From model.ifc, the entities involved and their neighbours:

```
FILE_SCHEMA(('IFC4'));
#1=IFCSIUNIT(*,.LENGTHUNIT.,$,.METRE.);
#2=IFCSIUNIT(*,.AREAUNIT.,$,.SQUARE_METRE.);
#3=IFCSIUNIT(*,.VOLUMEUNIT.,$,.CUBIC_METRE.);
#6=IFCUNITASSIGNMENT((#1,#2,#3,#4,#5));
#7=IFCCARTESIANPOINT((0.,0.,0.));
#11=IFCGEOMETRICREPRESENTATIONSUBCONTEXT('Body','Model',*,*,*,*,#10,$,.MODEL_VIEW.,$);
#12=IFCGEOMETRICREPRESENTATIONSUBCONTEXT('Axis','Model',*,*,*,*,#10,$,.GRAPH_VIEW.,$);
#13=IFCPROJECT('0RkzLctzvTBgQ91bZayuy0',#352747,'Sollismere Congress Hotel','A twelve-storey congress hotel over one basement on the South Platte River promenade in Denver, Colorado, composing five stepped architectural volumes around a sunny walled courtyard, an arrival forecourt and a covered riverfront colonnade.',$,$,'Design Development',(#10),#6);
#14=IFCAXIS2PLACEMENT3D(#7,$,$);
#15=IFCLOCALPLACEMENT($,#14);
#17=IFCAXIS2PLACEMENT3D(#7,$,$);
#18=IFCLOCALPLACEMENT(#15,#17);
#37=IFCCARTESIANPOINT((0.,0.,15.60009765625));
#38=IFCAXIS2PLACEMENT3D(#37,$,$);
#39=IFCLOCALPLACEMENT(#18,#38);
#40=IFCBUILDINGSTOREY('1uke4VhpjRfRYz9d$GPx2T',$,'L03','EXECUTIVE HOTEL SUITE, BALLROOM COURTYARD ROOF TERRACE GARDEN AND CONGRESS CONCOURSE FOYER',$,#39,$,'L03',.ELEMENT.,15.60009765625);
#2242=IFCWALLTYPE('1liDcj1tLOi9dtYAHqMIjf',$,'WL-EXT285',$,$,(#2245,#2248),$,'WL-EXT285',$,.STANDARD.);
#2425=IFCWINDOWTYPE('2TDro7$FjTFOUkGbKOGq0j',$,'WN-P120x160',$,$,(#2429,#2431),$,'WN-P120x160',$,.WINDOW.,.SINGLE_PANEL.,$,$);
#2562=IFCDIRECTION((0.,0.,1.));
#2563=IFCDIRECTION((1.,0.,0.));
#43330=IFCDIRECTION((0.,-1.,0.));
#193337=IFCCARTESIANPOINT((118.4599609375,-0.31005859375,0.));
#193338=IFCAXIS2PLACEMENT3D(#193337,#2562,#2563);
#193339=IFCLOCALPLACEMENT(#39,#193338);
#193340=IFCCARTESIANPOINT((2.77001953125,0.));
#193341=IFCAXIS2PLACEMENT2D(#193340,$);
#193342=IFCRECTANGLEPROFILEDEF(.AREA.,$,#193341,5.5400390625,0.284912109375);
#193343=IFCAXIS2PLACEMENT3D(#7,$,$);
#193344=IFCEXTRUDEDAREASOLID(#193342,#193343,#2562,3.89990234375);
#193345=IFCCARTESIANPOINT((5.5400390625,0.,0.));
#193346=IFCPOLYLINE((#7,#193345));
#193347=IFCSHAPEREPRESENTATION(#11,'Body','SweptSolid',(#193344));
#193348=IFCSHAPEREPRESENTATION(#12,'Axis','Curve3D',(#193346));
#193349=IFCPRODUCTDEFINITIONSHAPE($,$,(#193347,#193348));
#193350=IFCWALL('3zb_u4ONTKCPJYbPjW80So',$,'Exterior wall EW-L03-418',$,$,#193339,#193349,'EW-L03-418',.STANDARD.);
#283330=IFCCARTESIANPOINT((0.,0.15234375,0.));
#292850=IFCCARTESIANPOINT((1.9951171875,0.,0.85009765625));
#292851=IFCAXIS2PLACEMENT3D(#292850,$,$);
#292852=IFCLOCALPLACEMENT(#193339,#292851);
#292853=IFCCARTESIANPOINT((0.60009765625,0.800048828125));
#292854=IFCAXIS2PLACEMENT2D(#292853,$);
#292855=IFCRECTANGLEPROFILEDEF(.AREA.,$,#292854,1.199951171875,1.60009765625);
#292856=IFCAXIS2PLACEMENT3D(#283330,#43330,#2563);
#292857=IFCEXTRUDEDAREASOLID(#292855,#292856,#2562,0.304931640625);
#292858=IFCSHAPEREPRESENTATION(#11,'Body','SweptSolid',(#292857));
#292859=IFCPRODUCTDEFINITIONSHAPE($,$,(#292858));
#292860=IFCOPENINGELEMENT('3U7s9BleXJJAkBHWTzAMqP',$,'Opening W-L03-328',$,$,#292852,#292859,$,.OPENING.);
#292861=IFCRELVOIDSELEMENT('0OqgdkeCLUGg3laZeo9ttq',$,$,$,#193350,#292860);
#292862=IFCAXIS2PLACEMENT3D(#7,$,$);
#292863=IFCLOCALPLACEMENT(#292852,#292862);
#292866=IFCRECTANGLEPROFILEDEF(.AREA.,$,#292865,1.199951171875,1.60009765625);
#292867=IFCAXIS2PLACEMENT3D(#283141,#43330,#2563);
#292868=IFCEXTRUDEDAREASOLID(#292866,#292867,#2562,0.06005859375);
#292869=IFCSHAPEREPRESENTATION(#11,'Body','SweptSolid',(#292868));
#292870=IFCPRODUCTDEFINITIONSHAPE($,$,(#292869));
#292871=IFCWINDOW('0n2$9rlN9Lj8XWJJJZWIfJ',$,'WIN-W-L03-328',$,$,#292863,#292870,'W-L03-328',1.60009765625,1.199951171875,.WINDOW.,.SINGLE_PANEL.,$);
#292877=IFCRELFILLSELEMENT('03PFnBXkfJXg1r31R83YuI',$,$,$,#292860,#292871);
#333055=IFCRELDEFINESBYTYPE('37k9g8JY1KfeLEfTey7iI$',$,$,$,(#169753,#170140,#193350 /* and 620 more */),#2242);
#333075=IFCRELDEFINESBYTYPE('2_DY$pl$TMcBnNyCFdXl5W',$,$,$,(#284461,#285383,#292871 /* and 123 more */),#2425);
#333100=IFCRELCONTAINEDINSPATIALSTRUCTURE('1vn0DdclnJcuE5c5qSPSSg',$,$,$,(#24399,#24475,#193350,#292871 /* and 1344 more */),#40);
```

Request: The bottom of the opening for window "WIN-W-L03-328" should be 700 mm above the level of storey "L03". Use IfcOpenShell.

```python
import numpy as np
import ifcopenshell
import ifcopenshell.api.geometry
import ifcopenshell.geom
import ifcopenshell.util.element
import ifcopenshell.util.placement
import ifcopenshell.util.shape
import ifcopenshell.util.unit

model = ifcopenshell.open("model.ifc")
unit_scale = ifcopenshell.util.unit.calculate_unit_scale(model)

window = model.by_guid("0n2$9rlN9Lj8XWJJJZWIfJ")
opening = window.FillsVoids[0].RelatingOpeningElement
storey = ifcopenshell.util.element.get_container(window, ifc_class="IfcBuildingStorey")
level = ifcopenshell.util.placement.get_local_placement(storey.ObjectPlacement)[2, 3]

# The opening's origin need not be at the sill, so measure its lowest point.
shape = ifcopenshell.geom.create_shape(ifcopenshell.geom.settings(), opening)
bottom = ifcopenshell.util.shape.get_shape_bottom_elevation(shape, shape.geometry) / unit_scale
dz = level + 0.7 - bottom

shift = np.array([0.0, 0.0, dz])
# The window is placed relative to its opening, so it follows when the opening moves.
matrix = ifcopenshell.util.placement.get_local_placement(opening.ObjectPlacement)
matrix[:3, 3] += shift
ifcopenshell.api.geometry.edit_object_placement(
    model, product=opening, matrix=matrix, is_si=False, should_transform_children=True
)

print(f"moved by {dz * unit_scale:+.3f} m")

model.write("model_v2.ifc")
```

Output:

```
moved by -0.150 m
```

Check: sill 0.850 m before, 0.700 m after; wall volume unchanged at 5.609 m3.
